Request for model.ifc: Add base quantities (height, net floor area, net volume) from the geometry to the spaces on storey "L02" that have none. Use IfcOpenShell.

First a look at what the model holds.

```python
import ifcopenshell
import ifcopenshell.util.element
import ifcopenshell.util.unit

model = ifcopenshell.open("model.ifc")
print(model.schema)
for unit_type in ("LENGTHUNIT", "AREAUNIT", "VOLUMEUNIT"):
    print(unit_type, ifcopenshell.util.unit.calculate_unit_scale(model, unit_type))
storey = next(s for s in model.by_type("IfcBuildingStorey") if s.Name == "L02")
spaces = [e for e in ifcopenshell.util.element.get_decomposition(storey) if e.is_a("IfcSpace")]
for e in sorted(spaces, key=lambda e: e.id()):
    print(e.id(), e.is_a(), e.Name, list(ifcopenshell.util.element.get_psets(e, qtos_only=True)), sep=" | ")
```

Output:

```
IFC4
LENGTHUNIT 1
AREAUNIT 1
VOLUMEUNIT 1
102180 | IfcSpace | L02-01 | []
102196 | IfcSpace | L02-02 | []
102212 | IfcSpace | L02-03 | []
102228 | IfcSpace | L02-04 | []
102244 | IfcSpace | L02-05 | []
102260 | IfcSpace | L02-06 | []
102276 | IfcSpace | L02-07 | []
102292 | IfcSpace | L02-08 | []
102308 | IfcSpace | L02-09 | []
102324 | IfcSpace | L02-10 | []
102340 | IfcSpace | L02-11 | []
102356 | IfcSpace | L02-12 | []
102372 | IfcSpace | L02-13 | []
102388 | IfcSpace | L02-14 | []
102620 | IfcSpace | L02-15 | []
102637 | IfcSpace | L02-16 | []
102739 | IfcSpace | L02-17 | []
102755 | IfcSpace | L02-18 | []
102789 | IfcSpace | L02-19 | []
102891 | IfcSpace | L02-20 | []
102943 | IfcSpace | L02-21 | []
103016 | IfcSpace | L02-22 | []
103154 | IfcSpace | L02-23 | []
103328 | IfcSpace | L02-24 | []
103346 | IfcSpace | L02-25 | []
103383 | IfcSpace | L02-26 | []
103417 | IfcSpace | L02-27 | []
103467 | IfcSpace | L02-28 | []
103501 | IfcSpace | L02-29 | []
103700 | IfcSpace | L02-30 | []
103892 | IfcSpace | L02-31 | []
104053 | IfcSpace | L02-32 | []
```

```python
import ifcopenshell
import ifcopenshell.api.pset
import ifcopenshell.geom
import ifcopenshell.util.element
import ifcopenshell.util.shape
import ifcopenshell.util.unit

model = ifcopenshell.open("model.ifc")
unit_scale = ifcopenshell.util.unit.calculate_unit_scale(model)
area_scale = ifcopenshell.util.unit.calculate_unit_scale(model, "AREAUNIT")
volume_scale = ifcopenshell.util.unit.calculate_unit_scale(model, "VOLUMEUNIT")
settings = ifcopenshell.geom.settings()

storey = next(s for s in model.by_type("IfcBuildingStorey") if s.Name == "L02")
spaces = [e for e in ifcopenshell.util.element.get_decomposition(storey) if e.is_a("IfcSpace")]

for e in sorted(spaces, key=lambda e: e.id()):
    if ifcopenshell.util.element.get_psets(e, qtos_only=True, should_inherit=False):
        continue
    # Geometry comes back in metres, in the element's own axes.
    shape = ifcopenshell.geom.create_shape(settings, e)
    values = {
        "Height": ifcopenshell.util.shape.get_z(shape.geometry) / unit_scale,
        "NetFloorArea": ifcopenshell.util.shape.get_footprint_area(shape.geometry) / area_scale,
        "NetVolume": ifcopenshell.util.shape.get_volume(shape.geometry) / volume_scale,
    }
    qto = ifcopenshell.api.pset.add_qto(model, product=e, name="Qto_SpaceBaseQuantities")
    ifcopenshell.api.pset.edit_qto(model, qto=qto, properties=values)
    print(e.id(), {k: round(v, 3) for k, v in values.items()})

model.write("model_rev.ifc")
```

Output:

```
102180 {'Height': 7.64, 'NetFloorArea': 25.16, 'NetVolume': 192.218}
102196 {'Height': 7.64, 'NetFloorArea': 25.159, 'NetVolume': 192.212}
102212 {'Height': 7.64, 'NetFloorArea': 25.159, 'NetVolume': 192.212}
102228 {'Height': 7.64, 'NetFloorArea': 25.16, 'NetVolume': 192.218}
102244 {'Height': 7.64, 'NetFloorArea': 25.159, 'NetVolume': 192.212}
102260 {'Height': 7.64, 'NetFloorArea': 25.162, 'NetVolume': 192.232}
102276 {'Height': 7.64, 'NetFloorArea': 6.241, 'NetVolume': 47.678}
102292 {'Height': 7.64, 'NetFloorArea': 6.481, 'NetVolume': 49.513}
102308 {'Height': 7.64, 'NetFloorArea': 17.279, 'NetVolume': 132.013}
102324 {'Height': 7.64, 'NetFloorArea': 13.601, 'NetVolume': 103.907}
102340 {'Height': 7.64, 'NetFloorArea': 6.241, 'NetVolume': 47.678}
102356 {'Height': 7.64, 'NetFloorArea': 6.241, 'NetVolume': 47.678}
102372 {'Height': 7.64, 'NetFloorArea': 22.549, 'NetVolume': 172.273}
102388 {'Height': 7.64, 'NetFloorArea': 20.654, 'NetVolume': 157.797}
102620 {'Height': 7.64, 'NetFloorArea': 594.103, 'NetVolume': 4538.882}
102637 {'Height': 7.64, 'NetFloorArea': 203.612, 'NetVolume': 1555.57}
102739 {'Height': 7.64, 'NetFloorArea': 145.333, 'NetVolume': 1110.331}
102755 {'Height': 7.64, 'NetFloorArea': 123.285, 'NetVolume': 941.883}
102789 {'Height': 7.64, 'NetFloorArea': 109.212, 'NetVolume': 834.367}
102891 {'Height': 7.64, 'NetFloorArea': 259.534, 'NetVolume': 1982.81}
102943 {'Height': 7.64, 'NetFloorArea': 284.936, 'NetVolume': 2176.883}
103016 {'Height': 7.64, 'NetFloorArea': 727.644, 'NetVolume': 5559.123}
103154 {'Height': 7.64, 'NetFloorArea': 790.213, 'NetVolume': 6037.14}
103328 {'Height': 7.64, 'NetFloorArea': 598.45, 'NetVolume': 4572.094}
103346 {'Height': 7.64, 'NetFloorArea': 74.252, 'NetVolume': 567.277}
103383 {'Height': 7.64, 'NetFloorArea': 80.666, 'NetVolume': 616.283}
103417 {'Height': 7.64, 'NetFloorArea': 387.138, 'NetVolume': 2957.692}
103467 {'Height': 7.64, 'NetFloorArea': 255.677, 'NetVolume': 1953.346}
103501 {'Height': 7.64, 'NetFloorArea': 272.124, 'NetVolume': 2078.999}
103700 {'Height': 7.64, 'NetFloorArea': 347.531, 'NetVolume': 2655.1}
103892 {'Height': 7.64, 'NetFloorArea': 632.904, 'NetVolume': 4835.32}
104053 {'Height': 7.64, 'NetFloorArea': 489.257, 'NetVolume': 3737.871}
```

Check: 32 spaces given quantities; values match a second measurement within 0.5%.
